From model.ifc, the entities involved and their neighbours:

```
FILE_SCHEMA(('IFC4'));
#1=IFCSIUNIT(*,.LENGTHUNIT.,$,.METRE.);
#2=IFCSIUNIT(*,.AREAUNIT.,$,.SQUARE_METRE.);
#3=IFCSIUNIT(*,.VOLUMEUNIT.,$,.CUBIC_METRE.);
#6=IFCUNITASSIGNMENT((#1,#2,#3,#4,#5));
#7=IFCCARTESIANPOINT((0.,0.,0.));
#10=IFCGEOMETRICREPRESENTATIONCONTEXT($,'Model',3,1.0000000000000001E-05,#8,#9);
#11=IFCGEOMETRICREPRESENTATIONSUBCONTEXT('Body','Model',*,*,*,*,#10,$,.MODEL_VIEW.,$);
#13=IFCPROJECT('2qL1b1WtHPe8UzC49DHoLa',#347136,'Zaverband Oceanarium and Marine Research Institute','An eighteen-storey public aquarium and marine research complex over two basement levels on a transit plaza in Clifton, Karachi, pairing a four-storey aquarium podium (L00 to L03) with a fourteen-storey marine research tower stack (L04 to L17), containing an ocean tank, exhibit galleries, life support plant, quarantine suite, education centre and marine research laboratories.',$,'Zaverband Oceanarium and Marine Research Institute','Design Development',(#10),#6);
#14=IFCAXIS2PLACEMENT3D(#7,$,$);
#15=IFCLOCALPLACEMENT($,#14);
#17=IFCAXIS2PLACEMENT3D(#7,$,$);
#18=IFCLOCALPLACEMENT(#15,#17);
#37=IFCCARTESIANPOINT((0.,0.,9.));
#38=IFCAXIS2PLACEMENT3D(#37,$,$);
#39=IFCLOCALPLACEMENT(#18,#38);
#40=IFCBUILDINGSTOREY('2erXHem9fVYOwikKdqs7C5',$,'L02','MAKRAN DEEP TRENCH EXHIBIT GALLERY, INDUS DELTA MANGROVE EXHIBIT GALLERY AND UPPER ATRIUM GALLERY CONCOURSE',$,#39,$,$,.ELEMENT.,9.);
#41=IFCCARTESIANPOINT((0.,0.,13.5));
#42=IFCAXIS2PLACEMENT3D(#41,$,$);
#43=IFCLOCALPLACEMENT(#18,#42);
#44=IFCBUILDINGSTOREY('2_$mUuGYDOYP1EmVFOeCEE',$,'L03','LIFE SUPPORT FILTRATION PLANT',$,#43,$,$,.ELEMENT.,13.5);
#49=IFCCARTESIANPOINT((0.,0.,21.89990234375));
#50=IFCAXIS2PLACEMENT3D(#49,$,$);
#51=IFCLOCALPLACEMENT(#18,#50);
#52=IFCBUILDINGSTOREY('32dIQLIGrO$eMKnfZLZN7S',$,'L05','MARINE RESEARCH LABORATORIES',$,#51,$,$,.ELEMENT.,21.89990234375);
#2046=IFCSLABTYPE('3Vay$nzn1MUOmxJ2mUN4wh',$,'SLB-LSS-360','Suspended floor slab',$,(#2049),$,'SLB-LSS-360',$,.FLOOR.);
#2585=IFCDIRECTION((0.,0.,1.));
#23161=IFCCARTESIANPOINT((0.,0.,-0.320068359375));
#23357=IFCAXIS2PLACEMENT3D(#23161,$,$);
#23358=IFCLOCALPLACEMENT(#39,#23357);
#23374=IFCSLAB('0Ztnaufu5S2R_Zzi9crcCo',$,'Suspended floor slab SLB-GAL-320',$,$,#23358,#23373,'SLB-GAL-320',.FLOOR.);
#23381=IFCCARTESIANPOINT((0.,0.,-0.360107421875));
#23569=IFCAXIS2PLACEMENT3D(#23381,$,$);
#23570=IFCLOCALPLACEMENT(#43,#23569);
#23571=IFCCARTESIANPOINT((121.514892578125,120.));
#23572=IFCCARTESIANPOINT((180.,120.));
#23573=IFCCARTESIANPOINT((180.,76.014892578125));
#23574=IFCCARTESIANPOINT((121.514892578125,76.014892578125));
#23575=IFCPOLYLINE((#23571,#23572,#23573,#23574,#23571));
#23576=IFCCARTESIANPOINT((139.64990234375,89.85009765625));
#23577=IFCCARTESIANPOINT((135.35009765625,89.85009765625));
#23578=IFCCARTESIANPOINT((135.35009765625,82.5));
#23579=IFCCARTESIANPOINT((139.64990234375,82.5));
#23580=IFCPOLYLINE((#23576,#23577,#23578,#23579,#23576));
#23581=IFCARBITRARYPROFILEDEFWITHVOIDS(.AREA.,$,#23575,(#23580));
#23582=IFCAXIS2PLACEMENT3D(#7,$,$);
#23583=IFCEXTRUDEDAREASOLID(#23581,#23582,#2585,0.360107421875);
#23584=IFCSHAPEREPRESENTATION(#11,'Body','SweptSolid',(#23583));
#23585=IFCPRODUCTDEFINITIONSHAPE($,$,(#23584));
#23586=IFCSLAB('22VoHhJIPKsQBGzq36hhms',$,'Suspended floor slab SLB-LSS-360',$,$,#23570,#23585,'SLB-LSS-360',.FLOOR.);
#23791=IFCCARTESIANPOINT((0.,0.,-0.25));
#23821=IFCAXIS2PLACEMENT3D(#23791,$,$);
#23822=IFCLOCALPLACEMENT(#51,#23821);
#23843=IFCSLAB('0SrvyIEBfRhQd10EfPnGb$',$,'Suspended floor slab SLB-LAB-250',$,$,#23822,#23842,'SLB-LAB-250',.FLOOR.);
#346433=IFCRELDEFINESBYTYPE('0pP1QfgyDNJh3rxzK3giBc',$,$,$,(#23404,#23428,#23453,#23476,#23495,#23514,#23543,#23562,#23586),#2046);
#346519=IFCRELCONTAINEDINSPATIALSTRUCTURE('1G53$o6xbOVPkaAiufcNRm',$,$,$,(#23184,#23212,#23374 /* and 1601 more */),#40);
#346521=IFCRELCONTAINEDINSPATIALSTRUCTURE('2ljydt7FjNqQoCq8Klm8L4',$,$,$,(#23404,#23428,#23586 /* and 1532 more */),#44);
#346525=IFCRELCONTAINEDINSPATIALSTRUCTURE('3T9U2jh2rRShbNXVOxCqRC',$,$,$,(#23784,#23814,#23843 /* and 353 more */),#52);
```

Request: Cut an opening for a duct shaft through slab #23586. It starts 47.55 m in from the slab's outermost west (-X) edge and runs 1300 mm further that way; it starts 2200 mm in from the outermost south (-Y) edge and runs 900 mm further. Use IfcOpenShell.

```python
import numpy as np
import ifcopenshell
import ifcopenshell.api.feature
import ifcopenshell.api.geometry
import ifcopenshell.api.root
import ifcopenshell.geom
import ifcopenshell.util.placement
import ifcopenshell.util.representation
import ifcopenshell.util.shape
import ifcopenshell.util.unit

model = ifcopenshell.open("model.ifc")
unit_scale = ifcopenshell.util.unit.calculate_unit_scale(model)
settings = ifcopenshell.geom.settings()


def volume(element):
    """Net volume in cubic metres, openings subtracted."""
    shape = ifcopenshell.geom.create_shape(settings, element)
    return ifcopenshell.util.shape.get_volume(shape.geometry)


slab = model.by_guid("22VoHhJIPKsQBGzq36hhms")
before = volume(slab)

# Extent in the slab's own axes, in metres. The edges named are its -X and -Y sides.
slab_shape = ifcopenshell.geom.create_shape(settings, slab)
vertices = ifcopenshell.util.shape.get_vertices(slab_shape.geometry)
x_min, y_min, bottom = vertices.min(axis=0)
top = vertices[:, 2].max()

opening = ifcopenshell.api.root.create_entity(model, ifc_class="IfcOpeningElement", name="Duct shaft opening", predefined_type="OPENING")
context = ifcopenshell.util.representation.get_context(model, "Model", "Body", "MODEL_VIEW")
width, depth = 1.3, 0.9
outline = [(0.0, 0.0), (width, 0.0), (width, depth), (0.0, depth), (0.0, 0.0)]
# Overshoot both faces by 50 mm so the cut is clean.
shape = ifcopenshell.api.geometry.add_slab_representation(
    model, context=context, depth=top - bottom + 0.1, polyline=outline
)
ifcopenshell.api.geometry.assign_representation(model, product=opening, representation=shape)

matrix = ifcopenshell.util.placement.get_local_placement(slab.ObjectPlacement)
matrix[:, 3] = matrix @ np.append(np.array([x_min + 47.55, y_min + 2.2, bottom - 0.05]) / unit_scale, 1.0)
ifcopenshell.api.geometry.edit_object_placement(model, product=opening, matrix=matrix, is_si=False)
ifcopenshell.api.feature.add_feature(model, feature=opening, element=slab)

after = volume(slab)

print(f"slab volume {before:.3f} -> {after:.3f} m3")

model.write("model_edited.ifc")
```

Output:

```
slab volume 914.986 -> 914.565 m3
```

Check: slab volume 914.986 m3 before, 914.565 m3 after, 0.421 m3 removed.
